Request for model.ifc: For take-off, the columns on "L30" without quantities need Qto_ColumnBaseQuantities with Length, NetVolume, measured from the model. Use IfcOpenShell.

First a look at what the model holds.

```python
import ifcopenshell
import ifcopenshell.util.element
import ifcopenshell.util.unit

model = ifcopenshell.open("model.ifc")
print(model.schema)
for unit_type in ("LENGTHUNIT", "AREAUNIT", "VOLUMEUNIT"):
    print(unit_type, ifcopenshell.util.unit.calculate_unit_scale(model, unit_type))
storey = next(s for s in model.by_type("IfcBuildingStorey") if s.Name == "L30")
columns = [e for e in ifcopenshell.util.element.get_decomposition(storey) if e.is_a("IfcColumn")]
for e in sorted(columns, key=lambda e: e.id()):
    print(e.id(), e.is_a(), e.Name, list(ifcopenshell.util.element.get_psets(e, qtos_only=True)), sep=" | ")
```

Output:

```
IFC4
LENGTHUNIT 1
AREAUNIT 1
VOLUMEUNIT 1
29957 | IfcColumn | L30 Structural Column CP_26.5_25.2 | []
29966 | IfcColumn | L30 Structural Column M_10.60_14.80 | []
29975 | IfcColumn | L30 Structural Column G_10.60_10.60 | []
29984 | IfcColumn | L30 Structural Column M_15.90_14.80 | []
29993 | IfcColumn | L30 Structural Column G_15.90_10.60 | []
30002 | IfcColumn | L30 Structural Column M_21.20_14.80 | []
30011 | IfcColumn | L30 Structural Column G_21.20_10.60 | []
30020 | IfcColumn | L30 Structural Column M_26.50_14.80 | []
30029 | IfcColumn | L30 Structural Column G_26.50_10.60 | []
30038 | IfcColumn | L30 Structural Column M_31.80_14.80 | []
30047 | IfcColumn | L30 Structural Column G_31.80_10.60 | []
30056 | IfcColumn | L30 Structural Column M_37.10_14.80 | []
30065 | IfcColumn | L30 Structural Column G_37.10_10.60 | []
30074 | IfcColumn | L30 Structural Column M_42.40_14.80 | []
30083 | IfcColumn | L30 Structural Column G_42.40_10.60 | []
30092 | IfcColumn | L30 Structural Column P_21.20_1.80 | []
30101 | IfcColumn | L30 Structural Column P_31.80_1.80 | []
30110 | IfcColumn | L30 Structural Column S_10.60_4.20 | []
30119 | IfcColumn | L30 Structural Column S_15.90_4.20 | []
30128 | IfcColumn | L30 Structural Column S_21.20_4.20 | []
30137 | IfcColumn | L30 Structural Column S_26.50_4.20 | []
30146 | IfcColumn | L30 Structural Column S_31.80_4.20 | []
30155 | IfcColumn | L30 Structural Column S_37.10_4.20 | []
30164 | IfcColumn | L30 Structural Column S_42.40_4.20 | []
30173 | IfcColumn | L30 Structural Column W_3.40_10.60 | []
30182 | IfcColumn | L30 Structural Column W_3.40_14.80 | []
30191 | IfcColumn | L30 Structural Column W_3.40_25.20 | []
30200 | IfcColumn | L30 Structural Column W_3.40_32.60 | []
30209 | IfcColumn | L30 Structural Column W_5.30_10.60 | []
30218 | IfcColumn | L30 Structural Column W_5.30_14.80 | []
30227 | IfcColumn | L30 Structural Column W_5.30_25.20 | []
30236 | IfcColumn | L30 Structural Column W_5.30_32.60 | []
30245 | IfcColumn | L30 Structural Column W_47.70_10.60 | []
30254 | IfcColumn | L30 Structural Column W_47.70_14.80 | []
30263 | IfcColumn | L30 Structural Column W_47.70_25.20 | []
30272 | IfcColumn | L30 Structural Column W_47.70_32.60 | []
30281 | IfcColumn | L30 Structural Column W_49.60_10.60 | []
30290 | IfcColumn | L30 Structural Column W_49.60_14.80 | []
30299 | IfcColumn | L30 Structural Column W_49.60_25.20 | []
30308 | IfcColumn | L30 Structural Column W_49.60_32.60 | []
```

```python
import ifcopenshell
import ifcopenshell.api.pset
import ifcopenshell.geom
import ifcopenshell.util.element
import ifcopenshell.util.shape
import ifcopenshell.util.unit

model = ifcopenshell.open("model.ifc")
unit_scale = ifcopenshell.util.unit.calculate_unit_scale(model)
volume_scale = ifcopenshell.util.unit.calculate_unit_scale(model, "VOLUMEUNIT")
settings = ifcopenshell.geom.settings()

storey = next(s for s in model.by_type("IfcBuildingStorey") if s.Name == "L30")
columns = [e for e in ifcopenshell.util.element.get_decomposition(storey) if e.is_a("IfcColumn")]

for e in sorted(columns, key=lambda e: e.id()):
    if ifcopenshell.util.element.get_psets(e, qtos_only=True, should_inherit=False):
        continue
    # Geometry comes back in metres, in the element's own axes.
    shape = ifcopenshell.geom.create_shape(settings, e)
    values = {
        "Length": ifcopenshell.util.shape.get_z(shape.geometry) / unit_scale,
        "NetVolume": ifcopenshell.util.shape.get_volume(shape.geometry) / volume_scale,
    }
    qto = ifcopenshell.api.pset.add_qto(model, product=e, name="Qto_ColumnBaseQuantities")
    ifcopenshell.api.pset.edit_qto(model, qto=qto, properties=values)
    print(e.id(), {k: round(v, 3) for k, v in values.items()})

model.write("model_edited.ifc")
```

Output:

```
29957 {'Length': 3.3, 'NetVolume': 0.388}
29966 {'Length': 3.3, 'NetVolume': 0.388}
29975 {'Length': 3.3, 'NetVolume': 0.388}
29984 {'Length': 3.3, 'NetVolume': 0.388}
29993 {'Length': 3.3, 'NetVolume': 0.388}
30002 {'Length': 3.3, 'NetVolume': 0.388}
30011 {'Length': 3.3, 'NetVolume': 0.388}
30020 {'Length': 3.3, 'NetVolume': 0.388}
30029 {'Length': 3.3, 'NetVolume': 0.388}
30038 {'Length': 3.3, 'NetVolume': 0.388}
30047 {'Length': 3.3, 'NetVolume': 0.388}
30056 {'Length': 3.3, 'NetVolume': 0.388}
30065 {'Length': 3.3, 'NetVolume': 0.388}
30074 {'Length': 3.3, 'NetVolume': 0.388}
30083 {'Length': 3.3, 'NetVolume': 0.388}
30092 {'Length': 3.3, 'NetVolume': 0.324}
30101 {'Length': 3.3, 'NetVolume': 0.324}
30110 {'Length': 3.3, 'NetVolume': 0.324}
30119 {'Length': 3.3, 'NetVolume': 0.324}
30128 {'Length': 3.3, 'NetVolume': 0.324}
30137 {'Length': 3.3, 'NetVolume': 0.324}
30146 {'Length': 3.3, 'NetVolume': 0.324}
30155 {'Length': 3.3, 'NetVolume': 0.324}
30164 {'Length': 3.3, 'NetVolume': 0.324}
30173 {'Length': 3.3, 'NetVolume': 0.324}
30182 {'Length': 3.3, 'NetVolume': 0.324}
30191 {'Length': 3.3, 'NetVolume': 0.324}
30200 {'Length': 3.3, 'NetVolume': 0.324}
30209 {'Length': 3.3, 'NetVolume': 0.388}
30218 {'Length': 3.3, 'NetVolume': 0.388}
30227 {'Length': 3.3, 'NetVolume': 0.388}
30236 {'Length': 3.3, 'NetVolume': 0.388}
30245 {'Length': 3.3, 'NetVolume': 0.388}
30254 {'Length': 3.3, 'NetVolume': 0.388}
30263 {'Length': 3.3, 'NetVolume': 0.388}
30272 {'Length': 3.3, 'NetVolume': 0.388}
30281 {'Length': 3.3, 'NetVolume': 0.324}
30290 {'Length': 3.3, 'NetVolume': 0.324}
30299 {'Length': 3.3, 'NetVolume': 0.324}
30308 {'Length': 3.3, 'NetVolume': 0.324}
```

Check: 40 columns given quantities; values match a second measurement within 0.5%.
